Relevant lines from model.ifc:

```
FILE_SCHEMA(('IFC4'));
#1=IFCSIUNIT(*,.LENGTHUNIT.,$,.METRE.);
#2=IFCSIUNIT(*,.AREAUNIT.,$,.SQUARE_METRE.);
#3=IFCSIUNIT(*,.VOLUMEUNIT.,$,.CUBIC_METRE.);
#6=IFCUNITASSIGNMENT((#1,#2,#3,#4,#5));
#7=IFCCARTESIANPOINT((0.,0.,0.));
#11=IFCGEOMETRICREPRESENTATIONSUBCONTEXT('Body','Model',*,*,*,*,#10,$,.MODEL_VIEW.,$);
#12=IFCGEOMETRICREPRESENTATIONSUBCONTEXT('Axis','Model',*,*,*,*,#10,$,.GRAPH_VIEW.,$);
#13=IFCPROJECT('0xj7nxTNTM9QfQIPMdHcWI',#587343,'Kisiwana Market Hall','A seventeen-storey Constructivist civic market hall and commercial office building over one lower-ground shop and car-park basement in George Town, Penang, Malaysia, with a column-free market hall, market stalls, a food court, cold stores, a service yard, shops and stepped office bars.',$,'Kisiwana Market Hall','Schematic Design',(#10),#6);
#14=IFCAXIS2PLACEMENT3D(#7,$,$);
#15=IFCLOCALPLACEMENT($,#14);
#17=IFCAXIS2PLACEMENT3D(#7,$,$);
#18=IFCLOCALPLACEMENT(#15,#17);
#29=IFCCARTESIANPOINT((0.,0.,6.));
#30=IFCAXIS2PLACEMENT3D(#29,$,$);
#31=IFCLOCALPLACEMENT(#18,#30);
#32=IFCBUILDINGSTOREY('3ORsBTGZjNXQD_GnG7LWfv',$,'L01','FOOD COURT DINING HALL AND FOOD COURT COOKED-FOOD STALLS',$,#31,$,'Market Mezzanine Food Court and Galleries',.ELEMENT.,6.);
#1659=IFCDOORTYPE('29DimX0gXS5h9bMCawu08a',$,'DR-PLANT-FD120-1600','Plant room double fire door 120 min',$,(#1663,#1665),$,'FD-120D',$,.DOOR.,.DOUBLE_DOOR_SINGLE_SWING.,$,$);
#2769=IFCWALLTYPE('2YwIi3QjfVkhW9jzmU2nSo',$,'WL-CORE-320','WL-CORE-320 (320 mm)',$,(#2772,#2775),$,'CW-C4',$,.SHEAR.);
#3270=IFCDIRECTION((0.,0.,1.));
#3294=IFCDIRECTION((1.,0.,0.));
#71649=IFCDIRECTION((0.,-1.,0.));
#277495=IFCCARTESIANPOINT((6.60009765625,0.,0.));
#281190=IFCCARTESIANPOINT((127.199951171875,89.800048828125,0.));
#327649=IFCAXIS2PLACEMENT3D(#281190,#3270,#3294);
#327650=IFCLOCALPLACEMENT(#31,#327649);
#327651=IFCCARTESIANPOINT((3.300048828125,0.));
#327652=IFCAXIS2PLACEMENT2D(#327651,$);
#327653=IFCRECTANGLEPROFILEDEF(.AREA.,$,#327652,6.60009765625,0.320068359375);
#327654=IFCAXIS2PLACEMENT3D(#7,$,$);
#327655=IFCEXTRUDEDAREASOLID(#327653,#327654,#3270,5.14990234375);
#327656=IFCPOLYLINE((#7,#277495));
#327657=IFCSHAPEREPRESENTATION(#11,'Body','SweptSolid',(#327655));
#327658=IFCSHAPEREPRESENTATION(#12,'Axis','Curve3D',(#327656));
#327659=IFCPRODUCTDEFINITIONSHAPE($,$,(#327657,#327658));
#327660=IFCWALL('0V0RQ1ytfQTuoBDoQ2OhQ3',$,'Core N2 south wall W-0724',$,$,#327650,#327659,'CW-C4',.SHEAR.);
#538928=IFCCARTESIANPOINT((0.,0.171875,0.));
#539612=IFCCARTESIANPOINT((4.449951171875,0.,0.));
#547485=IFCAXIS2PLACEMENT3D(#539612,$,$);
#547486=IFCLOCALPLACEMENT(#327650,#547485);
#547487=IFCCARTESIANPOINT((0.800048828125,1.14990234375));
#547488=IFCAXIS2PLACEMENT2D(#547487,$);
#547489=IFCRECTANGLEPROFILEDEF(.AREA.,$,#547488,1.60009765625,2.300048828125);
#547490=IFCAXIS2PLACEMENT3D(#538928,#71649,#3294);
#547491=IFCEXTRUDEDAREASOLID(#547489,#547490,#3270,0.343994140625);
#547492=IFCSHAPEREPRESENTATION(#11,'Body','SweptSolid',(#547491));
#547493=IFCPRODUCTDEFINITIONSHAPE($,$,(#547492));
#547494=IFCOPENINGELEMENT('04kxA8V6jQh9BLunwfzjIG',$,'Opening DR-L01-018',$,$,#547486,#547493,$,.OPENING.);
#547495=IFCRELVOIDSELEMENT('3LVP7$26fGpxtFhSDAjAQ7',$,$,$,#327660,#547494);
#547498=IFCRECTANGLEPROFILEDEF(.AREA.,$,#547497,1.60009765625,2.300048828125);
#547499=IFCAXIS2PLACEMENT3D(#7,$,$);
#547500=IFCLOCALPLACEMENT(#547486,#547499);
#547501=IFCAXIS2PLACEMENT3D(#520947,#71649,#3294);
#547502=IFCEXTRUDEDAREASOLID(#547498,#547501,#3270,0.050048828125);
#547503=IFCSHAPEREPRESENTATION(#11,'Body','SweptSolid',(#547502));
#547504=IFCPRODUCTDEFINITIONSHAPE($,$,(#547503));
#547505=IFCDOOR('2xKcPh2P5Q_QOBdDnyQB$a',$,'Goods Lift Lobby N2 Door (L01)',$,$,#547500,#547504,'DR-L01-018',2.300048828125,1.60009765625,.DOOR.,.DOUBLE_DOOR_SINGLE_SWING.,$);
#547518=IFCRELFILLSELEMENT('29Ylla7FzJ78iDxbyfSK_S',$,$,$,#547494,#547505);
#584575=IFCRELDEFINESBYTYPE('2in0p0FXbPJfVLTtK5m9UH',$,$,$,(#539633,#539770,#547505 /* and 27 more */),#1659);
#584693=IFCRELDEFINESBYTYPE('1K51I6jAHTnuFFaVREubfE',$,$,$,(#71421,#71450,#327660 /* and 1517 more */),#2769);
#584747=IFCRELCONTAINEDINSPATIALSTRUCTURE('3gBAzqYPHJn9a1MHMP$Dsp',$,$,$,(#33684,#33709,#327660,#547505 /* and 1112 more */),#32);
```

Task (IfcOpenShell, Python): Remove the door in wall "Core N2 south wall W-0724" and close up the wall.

```python
import ifcopenshell
import ifcopenshell.api.feature
import ifcopenshell.api.root
import ifcopenshell.geom
import ifcopenshell.util.shape

model = ifcopenshell.open("model.ifc")
settings = ifcopenshell.geom.settings()


def volume(element):
    """Net volume in cubic metres, openings subtracted."""
    shape = ifcopenshell.geom.create_shape(settings, element)
    return ifcopenshell.util.shape.get_volume(shape.geometry)


door = model.by_guid("2xKcPh2P5Q_QOBdDnyQB$a")
opening = door.FillsVoids[0].RelatingOpeningElement
wall = opening.VoidsElements[0].RelatingBuildingElement
before = volume(wall)

ifcopenshell.api.root.remove_product(model, product=door)
ifcopenshell.api.feature.remove_feature(model, feature=opening)

after = volume(wall)

print(f"wall volume {before:.3f} -> {after:.3f} m3")

model.write("model_updated.ifc")
```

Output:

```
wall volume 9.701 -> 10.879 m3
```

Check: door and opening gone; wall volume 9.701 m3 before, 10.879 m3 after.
